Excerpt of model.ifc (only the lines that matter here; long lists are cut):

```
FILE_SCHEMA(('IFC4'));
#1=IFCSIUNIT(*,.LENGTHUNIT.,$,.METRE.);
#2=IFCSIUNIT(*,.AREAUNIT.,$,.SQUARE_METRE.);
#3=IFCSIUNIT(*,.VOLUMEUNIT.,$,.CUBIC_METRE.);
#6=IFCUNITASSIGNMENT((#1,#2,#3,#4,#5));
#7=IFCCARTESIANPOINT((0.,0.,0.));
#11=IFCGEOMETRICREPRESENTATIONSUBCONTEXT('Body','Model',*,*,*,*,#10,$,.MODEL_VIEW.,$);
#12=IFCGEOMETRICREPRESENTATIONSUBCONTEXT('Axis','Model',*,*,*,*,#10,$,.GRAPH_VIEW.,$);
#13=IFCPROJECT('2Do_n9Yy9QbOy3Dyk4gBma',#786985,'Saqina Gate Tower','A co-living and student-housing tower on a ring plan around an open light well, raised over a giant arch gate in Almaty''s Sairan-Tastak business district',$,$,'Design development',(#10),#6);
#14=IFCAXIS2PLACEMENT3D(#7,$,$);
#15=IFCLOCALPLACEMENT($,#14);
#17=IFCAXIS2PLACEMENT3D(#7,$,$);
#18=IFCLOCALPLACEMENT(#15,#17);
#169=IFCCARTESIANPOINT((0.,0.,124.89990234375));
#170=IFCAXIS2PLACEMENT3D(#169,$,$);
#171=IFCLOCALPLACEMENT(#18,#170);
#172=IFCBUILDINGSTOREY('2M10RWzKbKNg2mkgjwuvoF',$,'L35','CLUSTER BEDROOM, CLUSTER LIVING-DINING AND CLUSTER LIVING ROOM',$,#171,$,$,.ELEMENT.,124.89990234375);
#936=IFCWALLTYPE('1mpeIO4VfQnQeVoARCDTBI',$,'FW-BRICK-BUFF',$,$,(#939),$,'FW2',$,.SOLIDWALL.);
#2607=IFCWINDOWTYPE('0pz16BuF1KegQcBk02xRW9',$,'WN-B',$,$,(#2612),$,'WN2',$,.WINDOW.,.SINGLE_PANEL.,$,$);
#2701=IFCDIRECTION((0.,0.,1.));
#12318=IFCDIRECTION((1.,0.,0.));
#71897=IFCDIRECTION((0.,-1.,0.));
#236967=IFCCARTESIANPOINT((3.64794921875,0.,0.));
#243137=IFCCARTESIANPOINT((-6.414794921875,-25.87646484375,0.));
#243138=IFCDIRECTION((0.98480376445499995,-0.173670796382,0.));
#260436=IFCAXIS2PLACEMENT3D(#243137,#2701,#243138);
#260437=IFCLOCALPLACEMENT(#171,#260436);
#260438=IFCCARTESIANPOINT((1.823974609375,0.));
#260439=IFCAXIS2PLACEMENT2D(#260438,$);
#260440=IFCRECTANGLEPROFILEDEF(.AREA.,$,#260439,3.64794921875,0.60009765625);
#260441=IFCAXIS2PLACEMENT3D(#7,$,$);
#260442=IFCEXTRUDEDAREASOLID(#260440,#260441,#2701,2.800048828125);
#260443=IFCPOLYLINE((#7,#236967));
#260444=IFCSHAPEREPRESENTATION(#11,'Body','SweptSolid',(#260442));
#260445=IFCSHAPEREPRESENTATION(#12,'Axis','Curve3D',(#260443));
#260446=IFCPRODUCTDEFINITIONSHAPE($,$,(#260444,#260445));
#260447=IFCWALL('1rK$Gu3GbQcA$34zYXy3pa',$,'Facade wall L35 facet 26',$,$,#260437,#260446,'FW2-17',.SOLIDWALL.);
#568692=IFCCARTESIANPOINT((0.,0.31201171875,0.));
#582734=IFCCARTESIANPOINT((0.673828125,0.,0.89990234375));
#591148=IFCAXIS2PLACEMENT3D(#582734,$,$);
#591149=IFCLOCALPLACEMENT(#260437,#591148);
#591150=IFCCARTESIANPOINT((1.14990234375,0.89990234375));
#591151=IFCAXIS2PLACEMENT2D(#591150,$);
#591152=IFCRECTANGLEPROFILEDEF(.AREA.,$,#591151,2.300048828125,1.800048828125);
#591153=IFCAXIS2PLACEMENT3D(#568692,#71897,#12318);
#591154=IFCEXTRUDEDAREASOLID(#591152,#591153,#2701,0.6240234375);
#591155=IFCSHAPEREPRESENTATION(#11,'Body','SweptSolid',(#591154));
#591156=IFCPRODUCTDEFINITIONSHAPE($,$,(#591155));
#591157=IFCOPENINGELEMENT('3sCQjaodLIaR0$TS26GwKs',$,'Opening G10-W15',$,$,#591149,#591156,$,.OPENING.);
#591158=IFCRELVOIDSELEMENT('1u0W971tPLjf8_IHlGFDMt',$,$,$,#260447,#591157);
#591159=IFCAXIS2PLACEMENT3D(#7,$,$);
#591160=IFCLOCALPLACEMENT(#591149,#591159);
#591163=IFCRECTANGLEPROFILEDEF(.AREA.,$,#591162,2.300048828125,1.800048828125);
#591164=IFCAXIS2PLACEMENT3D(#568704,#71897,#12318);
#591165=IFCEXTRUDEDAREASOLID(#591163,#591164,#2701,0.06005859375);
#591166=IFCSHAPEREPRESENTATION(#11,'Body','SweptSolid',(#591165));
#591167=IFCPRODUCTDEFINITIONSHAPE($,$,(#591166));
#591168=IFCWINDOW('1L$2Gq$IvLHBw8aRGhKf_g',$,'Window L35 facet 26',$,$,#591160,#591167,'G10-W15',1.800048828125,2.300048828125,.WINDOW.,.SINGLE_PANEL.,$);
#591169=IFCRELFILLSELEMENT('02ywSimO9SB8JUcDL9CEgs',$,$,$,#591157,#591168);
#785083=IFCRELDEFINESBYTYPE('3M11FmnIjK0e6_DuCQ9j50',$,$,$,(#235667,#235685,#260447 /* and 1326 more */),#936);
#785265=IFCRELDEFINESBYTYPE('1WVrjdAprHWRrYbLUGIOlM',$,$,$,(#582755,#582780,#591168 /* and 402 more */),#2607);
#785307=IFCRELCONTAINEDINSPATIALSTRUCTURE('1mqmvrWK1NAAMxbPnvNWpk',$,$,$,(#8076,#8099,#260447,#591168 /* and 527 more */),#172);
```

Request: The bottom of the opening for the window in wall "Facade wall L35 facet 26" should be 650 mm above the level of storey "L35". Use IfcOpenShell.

```python
import numpy as np
import ifcopenshell
import ifcopenshell.api.geometry
import ifcopenshell.geom
import ifcopenshell.util.element
import ifcopenshell.util.placement
import ifcopenshell.util.shape
import ifcopenshell.util.unit

model = ifcopenshell.open("model.ifc")
unit_scale = ifcopenshell.util.unit.calculate_unit_scale(model)

window = model.by_id(591168)
opening = window.FillsVoids[0].RelatingOpeningElement
storey = ifcopenshell.util.element.get_container(window, ifc_class="IfcBuildingStorey")
level = ifcopenshell.util.placement.get_local_placement(storey.ObjectPlacement)[2, 3]

# The opening's origin need not be at the sill, so measure its lowest point.
shape = ifcopenshell.geom.create_shape(ifcopenshell.geom.settings(), opening)
bottom = ifcopenshell.util.shape.get_shape_bottom_elevation(shape, shape.geometry) / unit_scale
dz = level + 0.65 - bottom

shift = np.array([0.0, 0.0, dz])
# The window is placed relative to its opening, so it follows when the opening moves.
matrix = ifcopenshell.util.placement.get_local_placement(opening.ObjectPlacement)
matrix[:3, 3] += shift
ifcopenshell.api.geometry.edit_object_placement(
    model, product=opening, matrix=matrix, is_si=False, should_transform_children=True
)

print(f"moved by {dz * unit_scale:+.3f} m")

model.write("model_updated.ifc")
```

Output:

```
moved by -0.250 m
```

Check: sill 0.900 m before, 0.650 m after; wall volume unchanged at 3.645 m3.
